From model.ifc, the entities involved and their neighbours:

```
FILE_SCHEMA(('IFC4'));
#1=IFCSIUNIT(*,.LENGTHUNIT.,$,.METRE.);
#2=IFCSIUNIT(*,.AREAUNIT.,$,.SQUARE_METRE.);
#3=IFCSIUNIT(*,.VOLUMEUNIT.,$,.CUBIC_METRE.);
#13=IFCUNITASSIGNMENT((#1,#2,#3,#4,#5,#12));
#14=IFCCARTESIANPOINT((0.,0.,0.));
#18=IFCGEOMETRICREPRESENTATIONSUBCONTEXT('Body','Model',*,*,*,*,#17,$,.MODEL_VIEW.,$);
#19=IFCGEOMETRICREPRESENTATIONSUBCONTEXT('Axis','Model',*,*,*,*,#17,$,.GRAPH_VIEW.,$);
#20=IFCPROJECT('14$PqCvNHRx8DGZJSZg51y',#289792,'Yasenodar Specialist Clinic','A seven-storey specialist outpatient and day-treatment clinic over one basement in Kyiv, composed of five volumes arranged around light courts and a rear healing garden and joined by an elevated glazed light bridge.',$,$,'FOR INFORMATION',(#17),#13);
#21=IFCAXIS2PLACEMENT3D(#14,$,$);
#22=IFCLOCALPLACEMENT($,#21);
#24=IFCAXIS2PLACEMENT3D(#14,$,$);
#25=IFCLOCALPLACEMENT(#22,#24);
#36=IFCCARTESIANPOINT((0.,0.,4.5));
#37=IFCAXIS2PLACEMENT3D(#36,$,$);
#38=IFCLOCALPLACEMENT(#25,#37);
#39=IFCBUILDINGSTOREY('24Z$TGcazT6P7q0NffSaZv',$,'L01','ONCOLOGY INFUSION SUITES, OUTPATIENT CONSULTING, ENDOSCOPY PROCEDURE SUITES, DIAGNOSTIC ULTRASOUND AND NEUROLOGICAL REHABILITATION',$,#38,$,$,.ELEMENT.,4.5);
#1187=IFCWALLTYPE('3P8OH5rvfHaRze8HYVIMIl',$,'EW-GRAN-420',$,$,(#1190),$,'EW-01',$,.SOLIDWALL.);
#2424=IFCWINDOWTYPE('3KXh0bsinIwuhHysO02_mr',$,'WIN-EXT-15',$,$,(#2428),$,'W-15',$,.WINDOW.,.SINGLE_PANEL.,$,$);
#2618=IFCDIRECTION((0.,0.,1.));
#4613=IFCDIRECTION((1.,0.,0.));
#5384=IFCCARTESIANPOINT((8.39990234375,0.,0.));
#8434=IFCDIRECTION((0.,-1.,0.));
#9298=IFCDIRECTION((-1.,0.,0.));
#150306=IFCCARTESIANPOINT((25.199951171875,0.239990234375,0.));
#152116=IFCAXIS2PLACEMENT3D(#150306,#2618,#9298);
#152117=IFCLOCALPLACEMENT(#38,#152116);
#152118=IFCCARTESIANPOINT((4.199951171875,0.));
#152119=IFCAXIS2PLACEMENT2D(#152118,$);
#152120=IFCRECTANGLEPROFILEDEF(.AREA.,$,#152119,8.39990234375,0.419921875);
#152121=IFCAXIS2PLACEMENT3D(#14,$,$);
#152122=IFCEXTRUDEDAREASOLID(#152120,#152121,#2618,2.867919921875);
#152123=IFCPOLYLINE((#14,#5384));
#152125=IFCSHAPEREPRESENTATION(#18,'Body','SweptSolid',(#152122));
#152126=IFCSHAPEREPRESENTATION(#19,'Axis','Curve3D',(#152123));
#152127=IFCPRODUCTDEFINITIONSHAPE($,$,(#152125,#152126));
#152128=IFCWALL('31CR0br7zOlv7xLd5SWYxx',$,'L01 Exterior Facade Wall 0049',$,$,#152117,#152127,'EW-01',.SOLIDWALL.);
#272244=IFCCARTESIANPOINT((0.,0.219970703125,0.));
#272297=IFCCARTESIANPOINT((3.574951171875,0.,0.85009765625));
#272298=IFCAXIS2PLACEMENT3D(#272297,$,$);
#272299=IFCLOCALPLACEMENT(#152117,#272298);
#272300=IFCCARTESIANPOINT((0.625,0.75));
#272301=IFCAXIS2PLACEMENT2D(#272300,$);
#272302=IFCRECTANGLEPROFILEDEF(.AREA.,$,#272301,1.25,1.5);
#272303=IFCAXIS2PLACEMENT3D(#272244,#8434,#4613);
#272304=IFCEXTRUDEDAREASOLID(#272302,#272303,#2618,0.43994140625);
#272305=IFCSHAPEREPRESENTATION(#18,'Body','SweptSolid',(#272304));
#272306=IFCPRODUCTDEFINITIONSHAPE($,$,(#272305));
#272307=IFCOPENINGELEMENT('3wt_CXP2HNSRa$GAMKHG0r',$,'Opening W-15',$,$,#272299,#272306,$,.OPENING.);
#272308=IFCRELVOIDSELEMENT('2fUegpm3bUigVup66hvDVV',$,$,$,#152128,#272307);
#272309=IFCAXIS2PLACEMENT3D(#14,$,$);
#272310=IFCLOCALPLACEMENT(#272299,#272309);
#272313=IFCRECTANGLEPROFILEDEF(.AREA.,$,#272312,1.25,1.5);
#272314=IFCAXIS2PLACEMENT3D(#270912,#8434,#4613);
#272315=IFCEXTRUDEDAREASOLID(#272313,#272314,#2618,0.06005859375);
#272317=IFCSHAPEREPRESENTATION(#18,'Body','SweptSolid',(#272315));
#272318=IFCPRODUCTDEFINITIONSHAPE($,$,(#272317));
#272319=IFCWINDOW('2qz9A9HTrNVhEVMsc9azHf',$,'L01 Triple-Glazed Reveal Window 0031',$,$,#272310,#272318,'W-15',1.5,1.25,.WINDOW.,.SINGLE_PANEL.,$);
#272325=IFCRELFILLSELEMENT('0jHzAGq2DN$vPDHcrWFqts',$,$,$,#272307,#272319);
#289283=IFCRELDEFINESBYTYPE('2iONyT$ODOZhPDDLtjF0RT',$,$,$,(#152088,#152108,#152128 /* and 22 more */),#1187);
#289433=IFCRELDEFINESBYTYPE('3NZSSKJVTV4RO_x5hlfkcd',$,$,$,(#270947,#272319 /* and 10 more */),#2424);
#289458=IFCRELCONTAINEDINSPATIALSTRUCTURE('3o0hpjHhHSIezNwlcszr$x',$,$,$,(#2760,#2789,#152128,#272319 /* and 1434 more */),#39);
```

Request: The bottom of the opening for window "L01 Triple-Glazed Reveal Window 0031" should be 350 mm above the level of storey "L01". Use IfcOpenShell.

```python
import numpy as np
import ifcopenshell
import ifcopenshell.api.geometry
import ifcopenshell.geom
import ifcopenshell.util.element
import ifcopenshell.util.placement
import ifcopenshell.util.shape
import ifcopenshell.util.unit

model = ifcopenshell.open("model.ifc")
unit_scale = ifcopenshell.util.unit.calculate_unit_scale(model)

window = model.by_guid("2qz9A9HTrNVhEVMsc9azHf")
opening = window.FillsVoids[0].RelatingOpeningElement
storey = ifcopenshell.util.element.get_container(window, ifc_class="IfcBuildingStorey")
level = ifcopenshell.util.placement.get_local_placement(storey.ObjectPlacement)[2, 3]

# The opening's origin need not be at the sill, so measure its lowest point.
shape = ifcopenshell.geom.create_shape(ifcopenshell.geom.settings(), opening)
bottom = ifcopenshell.util.shape.get_shape_bottom_elevation(shape, shape.geometry) / unit_scale
dz = level + 0.35 / unit_scale - bottom

shift = np.array([0.0, 0.0, dz])
# The window is placed relative to its opening, so it follows when the opening moves.
matrix = ifcopenshell.util.placement.get_local_placement(opening.ObjectPlacement)
matrix[:3, 3] += shift
ifcopenshell.api.geometry.edit_object_placement(
    model, product=opening, matrix=matrix, is_si=False, should_transform_children=True
)

print(f"moved by {dz * unit_scale:+.3f} m")

model.write("model_edited.ifc")
```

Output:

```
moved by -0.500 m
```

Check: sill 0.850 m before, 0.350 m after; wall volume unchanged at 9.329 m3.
